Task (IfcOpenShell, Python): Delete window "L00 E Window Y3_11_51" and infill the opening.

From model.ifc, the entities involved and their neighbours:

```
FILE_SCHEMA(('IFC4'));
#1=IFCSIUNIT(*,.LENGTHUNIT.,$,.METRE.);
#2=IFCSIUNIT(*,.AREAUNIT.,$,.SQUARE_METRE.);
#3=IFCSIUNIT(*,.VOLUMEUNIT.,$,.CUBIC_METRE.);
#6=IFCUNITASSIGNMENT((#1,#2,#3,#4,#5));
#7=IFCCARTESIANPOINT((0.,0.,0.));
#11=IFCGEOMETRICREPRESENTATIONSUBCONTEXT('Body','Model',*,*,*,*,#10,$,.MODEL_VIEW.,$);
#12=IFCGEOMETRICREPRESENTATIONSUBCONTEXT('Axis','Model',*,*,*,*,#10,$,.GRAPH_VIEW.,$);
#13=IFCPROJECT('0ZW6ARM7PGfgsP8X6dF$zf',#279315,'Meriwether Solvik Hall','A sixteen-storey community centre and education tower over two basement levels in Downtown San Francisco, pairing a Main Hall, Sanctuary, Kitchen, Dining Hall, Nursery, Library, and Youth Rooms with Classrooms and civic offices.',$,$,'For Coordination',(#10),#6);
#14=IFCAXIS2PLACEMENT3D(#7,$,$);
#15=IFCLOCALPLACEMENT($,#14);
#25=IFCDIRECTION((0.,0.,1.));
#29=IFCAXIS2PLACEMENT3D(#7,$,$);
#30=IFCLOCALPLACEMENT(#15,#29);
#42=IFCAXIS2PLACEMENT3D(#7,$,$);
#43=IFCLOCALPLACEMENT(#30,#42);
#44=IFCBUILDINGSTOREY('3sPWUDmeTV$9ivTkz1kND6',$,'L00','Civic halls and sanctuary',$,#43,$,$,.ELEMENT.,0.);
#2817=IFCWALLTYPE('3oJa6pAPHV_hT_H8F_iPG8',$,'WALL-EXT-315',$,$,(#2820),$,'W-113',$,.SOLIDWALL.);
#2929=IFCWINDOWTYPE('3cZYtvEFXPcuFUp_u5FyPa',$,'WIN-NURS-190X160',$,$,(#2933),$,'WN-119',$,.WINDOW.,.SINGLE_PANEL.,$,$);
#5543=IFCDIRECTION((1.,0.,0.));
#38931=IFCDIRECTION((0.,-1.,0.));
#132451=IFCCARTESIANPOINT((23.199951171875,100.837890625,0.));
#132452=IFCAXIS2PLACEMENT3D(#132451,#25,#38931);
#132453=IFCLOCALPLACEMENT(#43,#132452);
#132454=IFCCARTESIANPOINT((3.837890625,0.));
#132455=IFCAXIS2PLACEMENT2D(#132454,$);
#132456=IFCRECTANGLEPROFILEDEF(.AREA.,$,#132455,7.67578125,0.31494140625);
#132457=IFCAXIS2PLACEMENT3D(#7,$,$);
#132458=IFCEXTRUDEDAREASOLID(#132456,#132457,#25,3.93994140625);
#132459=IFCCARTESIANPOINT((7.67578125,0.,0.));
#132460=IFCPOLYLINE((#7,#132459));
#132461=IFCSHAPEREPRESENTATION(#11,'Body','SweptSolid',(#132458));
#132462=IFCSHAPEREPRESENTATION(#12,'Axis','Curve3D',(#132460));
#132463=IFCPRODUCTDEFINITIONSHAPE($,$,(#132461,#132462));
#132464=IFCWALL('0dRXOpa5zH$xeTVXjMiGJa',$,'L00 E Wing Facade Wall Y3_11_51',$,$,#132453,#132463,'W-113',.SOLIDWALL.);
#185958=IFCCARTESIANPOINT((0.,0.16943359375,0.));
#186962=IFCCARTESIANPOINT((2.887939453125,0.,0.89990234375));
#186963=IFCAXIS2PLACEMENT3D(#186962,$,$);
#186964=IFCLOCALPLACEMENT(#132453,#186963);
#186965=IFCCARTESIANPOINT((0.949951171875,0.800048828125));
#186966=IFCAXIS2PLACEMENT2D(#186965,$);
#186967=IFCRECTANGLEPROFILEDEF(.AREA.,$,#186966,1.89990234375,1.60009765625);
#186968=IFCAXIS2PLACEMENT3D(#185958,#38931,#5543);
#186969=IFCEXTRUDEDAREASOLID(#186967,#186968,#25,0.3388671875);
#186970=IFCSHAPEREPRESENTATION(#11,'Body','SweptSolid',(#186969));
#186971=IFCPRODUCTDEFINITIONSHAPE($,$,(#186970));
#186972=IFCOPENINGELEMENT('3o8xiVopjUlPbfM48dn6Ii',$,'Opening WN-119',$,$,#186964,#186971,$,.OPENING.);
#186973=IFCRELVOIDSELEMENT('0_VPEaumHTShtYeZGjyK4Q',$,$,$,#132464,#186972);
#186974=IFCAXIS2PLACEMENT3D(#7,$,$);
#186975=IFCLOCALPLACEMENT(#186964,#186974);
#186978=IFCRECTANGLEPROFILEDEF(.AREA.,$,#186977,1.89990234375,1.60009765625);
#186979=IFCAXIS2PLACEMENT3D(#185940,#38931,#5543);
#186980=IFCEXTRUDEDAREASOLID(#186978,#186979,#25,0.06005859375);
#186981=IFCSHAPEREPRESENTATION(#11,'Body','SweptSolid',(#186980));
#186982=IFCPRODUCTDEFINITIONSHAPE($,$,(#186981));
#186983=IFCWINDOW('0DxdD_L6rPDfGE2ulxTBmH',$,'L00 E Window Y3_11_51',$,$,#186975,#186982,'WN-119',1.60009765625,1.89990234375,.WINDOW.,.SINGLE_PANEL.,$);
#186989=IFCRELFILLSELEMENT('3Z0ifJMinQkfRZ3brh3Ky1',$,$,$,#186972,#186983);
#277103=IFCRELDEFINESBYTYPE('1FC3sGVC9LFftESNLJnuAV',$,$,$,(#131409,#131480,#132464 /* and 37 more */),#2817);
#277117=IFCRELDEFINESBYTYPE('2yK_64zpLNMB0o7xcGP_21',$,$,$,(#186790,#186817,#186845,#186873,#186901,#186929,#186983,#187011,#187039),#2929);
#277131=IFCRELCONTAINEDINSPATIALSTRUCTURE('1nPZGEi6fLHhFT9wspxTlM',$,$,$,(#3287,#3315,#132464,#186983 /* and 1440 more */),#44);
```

```python
import ifcopenshell
import ifcopenshell.api.feature
import ifcopenshell.api.root
import ifcopenshell.geom
import ifcopenshell.util.shape

model = ifcopenshell.open("model.ifc")
settings = ifcopenshell.geom.settings()


def volume(element):
    """Net volume in cubic metres, openings subtracted."""
    shape = ifcopenshell.geom.create_shape(settings, element)
    return ifcopenshell.util.shape.get_volume(shape.geometry)


window = model.by_guid("0DxdD_L6rPDfGE2ulxTBmH")
opening = window.FillsVoids[0].RelatingOpeningElement
wall = opening.VoidsElements[0].RelatingBuildingElement
before = volume(wall)

ifcopenshell.api.root.remove_product(model, product=window)
ifcopenshell.api.feature.remove_feature(model, feature=opening)

after = volume(wall)

print(f"wall volume {before:.3f} -> {after:.3f} m3")

model.write("model_v2.ifc")
```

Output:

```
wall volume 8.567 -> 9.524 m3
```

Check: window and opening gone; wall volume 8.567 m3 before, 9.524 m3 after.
